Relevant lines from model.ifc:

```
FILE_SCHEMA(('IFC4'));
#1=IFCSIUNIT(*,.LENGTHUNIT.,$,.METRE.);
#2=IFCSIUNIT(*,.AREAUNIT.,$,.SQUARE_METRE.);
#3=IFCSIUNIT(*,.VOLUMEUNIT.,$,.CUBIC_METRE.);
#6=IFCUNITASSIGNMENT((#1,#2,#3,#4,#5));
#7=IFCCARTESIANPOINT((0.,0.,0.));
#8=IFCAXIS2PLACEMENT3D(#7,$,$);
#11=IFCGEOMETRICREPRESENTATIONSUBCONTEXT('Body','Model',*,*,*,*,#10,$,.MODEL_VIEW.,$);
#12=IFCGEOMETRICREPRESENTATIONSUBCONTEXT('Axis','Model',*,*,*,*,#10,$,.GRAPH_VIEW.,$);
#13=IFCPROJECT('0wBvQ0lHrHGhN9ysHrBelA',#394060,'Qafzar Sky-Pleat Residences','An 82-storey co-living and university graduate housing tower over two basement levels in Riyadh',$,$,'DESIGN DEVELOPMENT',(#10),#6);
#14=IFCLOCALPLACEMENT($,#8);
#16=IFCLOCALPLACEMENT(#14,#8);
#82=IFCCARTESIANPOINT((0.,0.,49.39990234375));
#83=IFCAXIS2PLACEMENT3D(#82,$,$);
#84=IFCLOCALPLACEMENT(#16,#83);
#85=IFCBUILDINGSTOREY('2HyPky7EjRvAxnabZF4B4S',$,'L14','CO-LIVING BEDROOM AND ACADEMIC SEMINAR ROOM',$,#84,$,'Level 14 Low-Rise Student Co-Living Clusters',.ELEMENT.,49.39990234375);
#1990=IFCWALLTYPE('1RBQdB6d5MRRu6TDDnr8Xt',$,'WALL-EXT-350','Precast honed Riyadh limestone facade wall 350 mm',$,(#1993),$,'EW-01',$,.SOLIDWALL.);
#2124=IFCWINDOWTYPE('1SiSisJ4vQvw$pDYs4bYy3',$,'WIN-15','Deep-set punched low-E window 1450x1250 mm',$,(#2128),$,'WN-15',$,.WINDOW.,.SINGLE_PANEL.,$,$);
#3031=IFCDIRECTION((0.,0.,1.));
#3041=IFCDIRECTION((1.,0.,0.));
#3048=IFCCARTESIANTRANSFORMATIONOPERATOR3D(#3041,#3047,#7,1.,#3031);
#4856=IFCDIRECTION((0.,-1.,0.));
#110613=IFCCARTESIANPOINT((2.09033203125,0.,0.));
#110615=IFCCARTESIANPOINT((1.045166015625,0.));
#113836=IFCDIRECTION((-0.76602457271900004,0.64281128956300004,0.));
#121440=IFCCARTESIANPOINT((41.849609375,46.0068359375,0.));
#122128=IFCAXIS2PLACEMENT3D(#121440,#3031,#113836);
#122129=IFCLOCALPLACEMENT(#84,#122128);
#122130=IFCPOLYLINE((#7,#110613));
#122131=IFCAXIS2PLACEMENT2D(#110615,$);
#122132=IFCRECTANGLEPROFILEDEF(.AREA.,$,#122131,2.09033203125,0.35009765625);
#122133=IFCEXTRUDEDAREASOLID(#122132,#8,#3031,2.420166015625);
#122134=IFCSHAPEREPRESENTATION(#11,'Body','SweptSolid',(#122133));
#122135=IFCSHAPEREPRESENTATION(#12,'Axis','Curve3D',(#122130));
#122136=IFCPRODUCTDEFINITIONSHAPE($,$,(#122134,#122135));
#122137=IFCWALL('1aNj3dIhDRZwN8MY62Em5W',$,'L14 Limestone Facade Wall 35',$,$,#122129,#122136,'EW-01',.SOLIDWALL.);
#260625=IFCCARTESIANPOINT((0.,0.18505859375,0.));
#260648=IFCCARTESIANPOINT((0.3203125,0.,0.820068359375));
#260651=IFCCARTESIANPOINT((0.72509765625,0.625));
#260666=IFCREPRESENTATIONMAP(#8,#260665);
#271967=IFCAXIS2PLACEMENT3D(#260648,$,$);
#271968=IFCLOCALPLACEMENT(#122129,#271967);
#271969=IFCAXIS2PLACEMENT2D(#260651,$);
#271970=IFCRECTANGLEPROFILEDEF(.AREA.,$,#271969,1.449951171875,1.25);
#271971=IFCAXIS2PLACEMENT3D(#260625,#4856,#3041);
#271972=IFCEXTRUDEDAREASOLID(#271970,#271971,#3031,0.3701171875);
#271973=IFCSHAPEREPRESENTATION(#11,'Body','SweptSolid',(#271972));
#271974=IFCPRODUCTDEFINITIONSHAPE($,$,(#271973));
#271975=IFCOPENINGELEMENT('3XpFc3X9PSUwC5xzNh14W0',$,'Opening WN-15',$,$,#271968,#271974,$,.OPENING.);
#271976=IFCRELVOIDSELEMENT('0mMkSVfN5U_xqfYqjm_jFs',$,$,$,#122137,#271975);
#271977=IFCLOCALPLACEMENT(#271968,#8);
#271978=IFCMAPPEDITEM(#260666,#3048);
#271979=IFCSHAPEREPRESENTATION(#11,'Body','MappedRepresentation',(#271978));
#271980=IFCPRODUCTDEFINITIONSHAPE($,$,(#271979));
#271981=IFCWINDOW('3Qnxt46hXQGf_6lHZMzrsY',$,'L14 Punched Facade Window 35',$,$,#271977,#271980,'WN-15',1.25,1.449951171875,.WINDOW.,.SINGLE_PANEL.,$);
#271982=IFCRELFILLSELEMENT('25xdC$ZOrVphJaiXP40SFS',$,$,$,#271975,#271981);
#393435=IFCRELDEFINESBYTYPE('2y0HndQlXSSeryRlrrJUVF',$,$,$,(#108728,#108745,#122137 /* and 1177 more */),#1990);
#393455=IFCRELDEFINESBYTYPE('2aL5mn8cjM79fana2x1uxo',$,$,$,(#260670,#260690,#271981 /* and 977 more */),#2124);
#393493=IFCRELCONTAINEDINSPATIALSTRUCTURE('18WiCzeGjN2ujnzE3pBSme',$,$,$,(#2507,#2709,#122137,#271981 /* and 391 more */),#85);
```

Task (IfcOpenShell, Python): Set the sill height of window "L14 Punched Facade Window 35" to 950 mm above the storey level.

```python
import numpy as np
import ifcopenshell
import ifcopenshell.api.geometry
import ifcopenshell.geom
import ifcopenshell.util.element
import ifcopenshell.util.placement
import ifcopenshell.util.shape
import ifcopenshell.util.unit

model = ifcopenshell.open("model.ifc")
unit_scale = ifcopenshell.util.unit.calculate_unit_scale(model)

window = model.by_guid("3Qnxt46hXQGf_6lHZMzrsY")
opening = window.FillsVoids[0].RelatingOpeningElement
storey = ifcopenshell.util.element.get_container(window, ifc_class="IfcBuildingStorey")
level = ifcopenshell.util.placement.get_local_placement(storey.ObjectPlacement)[2, 3]

# The opening's origin need not be at the sill, so measure its lowest point.
shape = ifcopenshell.geom.create_shape(ifcopenshell.geom.settings(), opening)
bottom = ifcopenshell.util.shape.get_shape_bottom_elevation(shape, shape.geometry) / unit_scale
dz = level + 0.95 - bottom

shift = np.array([0.0, 0.0, dz])
# The window is placed relative to its opening, so it follows when the opening moves.
matrix = ifcopenshell.util.placement.get_local_placement(opening.ObjectPlacement)
matrix[:3, 3] += shift
ifcopenshell.api.geometry.edit_object_placement(
    model, product=opening, matrix=matrix, is_si=False, should_transform_children=True
)

print(f"moved by {dz * unit_scale:+.3f} m")

model.write("model_v2.ifc")
```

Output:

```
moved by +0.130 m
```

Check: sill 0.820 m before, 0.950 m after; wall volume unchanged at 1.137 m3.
